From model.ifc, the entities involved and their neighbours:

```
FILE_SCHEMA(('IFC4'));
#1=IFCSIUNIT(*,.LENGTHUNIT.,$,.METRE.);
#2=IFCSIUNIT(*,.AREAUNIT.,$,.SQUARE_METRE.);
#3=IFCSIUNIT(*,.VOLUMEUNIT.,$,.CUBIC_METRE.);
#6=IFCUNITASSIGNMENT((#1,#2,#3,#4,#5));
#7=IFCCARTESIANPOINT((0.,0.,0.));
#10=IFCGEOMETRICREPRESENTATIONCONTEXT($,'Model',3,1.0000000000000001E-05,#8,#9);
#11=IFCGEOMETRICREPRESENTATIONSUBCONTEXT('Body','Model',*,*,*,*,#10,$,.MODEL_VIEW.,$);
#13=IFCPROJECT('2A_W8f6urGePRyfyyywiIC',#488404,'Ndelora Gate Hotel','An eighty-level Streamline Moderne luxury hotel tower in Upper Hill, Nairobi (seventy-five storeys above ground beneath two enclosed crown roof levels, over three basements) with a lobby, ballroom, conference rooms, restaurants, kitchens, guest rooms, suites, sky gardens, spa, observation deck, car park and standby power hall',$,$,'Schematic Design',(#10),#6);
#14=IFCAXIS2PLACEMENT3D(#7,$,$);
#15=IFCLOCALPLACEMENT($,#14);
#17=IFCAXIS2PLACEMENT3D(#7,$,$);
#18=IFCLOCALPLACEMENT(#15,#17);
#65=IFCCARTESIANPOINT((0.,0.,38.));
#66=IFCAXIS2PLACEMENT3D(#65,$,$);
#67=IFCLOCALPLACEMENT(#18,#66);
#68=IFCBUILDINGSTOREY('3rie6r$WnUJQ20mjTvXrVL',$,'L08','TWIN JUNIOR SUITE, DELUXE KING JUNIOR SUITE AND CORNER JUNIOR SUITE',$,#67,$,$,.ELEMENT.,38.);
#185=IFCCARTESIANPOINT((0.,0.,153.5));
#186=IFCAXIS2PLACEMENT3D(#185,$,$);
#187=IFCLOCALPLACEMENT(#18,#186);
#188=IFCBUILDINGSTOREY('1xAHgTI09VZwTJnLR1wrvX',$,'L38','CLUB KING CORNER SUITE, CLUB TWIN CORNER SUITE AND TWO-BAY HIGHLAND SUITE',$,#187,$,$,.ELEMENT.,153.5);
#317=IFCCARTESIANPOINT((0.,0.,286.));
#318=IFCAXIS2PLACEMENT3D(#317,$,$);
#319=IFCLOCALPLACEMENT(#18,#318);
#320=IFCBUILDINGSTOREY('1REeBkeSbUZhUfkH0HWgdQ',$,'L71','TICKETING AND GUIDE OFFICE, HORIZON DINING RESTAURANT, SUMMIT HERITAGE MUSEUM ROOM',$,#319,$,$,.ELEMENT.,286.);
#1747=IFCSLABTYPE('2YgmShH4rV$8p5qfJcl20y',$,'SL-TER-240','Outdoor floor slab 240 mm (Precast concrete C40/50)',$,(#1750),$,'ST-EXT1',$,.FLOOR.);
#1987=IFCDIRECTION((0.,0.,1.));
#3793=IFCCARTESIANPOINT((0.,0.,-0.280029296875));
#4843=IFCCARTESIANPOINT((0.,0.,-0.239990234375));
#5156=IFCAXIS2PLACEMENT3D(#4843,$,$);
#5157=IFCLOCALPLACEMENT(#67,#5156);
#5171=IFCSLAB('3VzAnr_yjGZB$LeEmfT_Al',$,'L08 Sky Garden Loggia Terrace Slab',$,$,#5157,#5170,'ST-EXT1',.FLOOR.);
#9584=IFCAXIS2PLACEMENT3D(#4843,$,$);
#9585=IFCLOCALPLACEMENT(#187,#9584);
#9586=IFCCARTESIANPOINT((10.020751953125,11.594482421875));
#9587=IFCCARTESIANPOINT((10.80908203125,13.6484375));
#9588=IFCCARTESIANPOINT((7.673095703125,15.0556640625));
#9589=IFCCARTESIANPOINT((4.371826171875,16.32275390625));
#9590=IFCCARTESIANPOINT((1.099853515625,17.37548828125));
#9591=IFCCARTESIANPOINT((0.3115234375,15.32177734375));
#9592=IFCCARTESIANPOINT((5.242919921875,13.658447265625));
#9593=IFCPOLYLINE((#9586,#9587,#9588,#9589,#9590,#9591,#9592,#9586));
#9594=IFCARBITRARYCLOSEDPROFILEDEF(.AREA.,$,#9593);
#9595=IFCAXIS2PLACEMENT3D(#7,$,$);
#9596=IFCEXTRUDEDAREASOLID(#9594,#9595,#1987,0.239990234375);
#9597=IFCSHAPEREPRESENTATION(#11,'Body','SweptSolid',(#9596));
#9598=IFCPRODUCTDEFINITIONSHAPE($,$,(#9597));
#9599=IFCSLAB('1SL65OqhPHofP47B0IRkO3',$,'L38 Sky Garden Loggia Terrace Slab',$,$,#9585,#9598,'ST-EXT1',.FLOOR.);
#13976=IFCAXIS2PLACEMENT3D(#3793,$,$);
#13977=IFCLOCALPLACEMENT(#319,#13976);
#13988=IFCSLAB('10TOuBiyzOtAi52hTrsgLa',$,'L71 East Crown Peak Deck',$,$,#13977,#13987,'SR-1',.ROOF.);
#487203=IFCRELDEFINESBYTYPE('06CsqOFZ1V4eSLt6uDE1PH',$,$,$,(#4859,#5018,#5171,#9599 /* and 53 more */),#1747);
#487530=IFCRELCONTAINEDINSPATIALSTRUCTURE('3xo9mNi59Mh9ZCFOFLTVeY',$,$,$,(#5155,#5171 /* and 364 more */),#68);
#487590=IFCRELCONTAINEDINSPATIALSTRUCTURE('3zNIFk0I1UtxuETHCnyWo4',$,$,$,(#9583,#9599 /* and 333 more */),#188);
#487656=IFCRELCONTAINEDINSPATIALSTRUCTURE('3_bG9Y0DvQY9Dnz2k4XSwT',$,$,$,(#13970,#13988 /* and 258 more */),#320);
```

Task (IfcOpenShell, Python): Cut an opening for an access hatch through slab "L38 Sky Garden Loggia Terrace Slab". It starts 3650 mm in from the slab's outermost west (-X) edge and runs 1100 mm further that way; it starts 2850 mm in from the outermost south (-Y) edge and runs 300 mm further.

```python
import numpy as np
import ifcopenshell
import ifcopenshell.api.feature
import ifcopenshell.api.geometry
import ifcopenshell.api.root
import ifcopenshell.geom
import ifcopenshell.util.placement
import ifcopenshell.util.representation
import ifcopenshell.util.shape
import ifcopenshell.util.unit

model = ifcopenshell.open("model.ifc")
unit_scale = ifcopenshell.util.unit.calculate_unit_scale(model)
settings = ifcopenshell.geom.settings()


def volume(element):
    """Net volume in cubic metres, openings subtracted."""
    shape = ifcopenshell.geom.create_shape(settings, element)
    return ifcopenshell.util.shape.get_volume(shape.geometry)


slab = model.by_id(9599)
before = volume(slab)

# Extent in the slab's own axes, in metres. The edges named are its -X and -Y sides.
slab_shape = ifcopenshell.geom.create_shape(settings, slab)
vertices = ifcopenshell.util.shape.get_vertices(slab_shape.geometry)
x_min, y_min, bottom = vertices.min(axis=0)
top = vertices[:, 2].max()

opening = ifcopenshell.api.root.create_entity(model, ifc_class="IfcOpeningElement", name="Access hatch opening", predefined_type="OPENING")
context = ifcopenshell.util.representation.get_context(model, "Model", "Body", "MODEL_VIEW")
width, depth = 1.1, 0.3
outline = [(0.0, 0.0), (width, 0.0), (width, depth), (0.0, depth), (0.0, 0.0)]
# Overshoot both faces by 50 mm so the cut is clean.
shape = ifcopenshell.api.geometry.add_slab_representation(
    model, context=context, depth=top - bottom + 0.1, polyline=outline
)
ifcopenshell.api.geometry.assign_representation(model, product=opening, representation=shape)

matrix = ifcopenshell.util.placement.get_local_placement(slab.ObjectPlacement)
matrix[:, 3] = matrix @ np.append(np.array([x_min + 3.65, y_min + 2.85, bottom - 0.05]) / unit_scale, 1.0)
ifcopenshell.api.geometry.edit_object_placement(model, product=opening, matrix=matrix, is_si=False)
ifcopenshell.api.feature.add_feature(model, feature=opening, element=slab)

after = volume(slab)

print(f"slab volume {before:.3f} -> {after:.3f} m3")

model.write("model_rev.ifc")
```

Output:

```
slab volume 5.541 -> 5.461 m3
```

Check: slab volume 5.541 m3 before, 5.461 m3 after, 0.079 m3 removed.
